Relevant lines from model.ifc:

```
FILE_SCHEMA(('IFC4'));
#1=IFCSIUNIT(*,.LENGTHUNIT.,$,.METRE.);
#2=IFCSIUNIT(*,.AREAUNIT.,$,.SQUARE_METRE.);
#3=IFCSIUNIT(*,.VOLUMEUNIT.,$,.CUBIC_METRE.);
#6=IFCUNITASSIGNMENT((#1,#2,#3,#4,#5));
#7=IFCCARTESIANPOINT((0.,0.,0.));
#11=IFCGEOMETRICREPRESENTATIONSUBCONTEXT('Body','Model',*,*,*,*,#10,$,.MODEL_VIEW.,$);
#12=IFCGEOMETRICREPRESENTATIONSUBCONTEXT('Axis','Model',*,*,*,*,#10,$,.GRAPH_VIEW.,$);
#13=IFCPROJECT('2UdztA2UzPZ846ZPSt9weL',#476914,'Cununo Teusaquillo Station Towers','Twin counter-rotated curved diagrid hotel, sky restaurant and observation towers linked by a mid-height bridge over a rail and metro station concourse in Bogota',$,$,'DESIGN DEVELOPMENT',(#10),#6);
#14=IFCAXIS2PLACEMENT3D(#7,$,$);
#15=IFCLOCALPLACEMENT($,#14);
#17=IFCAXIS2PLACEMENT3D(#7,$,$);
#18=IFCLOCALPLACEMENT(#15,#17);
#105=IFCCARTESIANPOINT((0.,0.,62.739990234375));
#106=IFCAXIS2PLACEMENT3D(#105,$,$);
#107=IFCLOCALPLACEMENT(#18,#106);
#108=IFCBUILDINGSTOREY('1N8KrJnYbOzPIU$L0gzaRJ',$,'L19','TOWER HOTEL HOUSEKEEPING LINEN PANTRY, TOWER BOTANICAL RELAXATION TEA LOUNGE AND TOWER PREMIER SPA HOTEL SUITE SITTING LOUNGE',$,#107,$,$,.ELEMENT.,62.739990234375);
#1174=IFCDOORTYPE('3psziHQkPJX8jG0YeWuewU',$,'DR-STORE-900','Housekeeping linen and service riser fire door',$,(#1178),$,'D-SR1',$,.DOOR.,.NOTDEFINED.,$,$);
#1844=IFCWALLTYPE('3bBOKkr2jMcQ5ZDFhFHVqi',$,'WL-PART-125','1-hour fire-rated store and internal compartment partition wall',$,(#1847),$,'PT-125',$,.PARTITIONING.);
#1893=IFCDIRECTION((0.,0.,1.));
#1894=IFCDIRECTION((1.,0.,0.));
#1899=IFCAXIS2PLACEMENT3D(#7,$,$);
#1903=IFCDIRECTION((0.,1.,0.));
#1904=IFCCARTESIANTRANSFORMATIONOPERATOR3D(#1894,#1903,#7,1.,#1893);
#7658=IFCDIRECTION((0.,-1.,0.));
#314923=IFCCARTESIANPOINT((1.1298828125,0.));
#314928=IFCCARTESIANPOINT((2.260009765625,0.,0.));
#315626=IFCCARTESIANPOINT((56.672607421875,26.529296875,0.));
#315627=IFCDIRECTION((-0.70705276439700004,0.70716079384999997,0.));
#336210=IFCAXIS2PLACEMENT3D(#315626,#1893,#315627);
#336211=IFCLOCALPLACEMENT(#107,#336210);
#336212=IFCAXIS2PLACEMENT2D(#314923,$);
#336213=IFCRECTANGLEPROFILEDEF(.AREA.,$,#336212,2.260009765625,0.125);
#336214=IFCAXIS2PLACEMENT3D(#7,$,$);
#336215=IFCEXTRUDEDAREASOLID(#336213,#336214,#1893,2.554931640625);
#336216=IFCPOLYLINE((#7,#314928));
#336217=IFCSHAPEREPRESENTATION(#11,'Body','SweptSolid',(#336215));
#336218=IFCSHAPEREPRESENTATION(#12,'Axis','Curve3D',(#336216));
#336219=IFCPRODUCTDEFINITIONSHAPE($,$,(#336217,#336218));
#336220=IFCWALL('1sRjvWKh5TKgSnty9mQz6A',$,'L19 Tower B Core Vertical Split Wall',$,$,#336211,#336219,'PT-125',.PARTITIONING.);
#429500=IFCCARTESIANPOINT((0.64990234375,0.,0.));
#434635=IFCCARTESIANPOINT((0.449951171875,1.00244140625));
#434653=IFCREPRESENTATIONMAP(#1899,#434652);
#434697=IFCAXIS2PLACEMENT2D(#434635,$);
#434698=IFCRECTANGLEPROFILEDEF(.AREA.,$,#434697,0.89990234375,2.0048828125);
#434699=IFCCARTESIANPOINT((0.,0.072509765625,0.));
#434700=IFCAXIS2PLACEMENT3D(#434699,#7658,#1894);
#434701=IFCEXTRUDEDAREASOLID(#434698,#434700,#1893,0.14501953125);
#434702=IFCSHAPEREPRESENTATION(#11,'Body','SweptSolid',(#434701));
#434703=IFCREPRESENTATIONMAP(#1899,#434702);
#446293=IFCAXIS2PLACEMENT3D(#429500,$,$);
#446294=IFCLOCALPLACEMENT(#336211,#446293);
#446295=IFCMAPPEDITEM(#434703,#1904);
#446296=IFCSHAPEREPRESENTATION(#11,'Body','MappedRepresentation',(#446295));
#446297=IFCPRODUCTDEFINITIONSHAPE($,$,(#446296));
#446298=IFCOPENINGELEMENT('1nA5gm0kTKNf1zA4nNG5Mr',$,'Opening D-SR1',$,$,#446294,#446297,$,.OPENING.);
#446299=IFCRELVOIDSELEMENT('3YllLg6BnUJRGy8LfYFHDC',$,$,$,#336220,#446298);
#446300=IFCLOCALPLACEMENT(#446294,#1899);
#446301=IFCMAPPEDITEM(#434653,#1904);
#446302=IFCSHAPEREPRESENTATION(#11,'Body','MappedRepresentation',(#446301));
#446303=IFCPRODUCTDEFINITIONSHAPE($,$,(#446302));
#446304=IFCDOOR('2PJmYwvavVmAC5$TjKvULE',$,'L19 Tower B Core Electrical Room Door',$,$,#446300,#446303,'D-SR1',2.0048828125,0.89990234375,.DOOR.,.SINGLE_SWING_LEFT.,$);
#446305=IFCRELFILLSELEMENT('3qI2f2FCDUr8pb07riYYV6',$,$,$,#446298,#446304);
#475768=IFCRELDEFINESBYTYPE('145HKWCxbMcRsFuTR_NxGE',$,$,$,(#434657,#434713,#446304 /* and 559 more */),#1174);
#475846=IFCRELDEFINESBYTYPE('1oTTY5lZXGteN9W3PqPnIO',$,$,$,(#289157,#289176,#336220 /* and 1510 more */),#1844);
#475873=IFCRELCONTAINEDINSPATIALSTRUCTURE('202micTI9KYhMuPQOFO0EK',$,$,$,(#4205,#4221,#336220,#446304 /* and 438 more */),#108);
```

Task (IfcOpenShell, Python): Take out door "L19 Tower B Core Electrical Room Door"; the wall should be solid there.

```python
import ifcopenshell
import ifcopenshell.api.feature
import ifcopenshell.api.root
import ifcopenshell.geom
import ifcopenshell.util.shape

model = ifcopenshell.open("model.ifc")
settings = ifcopenshell.geom.settings()


def volume(element):
    """Net volume in cubic metres, openings subtracted."""
    shape = ifcopenshell.geom.create_shape(settings, element)
    return ifcopenshell.util.shape.get_volume(shape.geometry)


door = model.by_id(446304)
opening = door.FillsVoids[0].RelatingOpeningElement
wall = opening.VoidsElements[0].RelatingBuildingElement
before = volume(wall)

ifcopenshell.api.root.remove_product(model, product=door)
ifcopenshell.api.feature.remove_feature(model, feature=opening)

after = volume(wall)

print(f"wall volume {before:.3f} -> {after:.3f} m3")

model.write("model_rev.ifc")
```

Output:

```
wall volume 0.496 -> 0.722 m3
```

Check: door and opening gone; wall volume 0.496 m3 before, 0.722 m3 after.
